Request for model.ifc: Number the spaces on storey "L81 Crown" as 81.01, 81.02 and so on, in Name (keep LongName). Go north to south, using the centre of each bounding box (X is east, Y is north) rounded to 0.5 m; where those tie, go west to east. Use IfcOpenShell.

First a look at what the model holds.

```python
import ifcopenshell
import ifcopenshell.util.element
import ifcopenshell.util.placement

model = ifcopenshell.open("model.ifc")
print(model.schema)
storey = next(s for s in model.by_type("IfcBuildingStorey") if s.Name == "L81 Crown")
spaces = [e for e in ifcopenshell.util.element.get_decomposition(storey) if e.is_a("IfcSpace")]
for e in sorted(spaces, key=lambda e: e.id()):
    origin = ifcopenshell.util.placement.get_local_placement(e.ObjectPlacement)[:3, 3]
    print(e.id(), e.Name, e.LongName, origin.round(2) + 0.0, sep=" | ")
```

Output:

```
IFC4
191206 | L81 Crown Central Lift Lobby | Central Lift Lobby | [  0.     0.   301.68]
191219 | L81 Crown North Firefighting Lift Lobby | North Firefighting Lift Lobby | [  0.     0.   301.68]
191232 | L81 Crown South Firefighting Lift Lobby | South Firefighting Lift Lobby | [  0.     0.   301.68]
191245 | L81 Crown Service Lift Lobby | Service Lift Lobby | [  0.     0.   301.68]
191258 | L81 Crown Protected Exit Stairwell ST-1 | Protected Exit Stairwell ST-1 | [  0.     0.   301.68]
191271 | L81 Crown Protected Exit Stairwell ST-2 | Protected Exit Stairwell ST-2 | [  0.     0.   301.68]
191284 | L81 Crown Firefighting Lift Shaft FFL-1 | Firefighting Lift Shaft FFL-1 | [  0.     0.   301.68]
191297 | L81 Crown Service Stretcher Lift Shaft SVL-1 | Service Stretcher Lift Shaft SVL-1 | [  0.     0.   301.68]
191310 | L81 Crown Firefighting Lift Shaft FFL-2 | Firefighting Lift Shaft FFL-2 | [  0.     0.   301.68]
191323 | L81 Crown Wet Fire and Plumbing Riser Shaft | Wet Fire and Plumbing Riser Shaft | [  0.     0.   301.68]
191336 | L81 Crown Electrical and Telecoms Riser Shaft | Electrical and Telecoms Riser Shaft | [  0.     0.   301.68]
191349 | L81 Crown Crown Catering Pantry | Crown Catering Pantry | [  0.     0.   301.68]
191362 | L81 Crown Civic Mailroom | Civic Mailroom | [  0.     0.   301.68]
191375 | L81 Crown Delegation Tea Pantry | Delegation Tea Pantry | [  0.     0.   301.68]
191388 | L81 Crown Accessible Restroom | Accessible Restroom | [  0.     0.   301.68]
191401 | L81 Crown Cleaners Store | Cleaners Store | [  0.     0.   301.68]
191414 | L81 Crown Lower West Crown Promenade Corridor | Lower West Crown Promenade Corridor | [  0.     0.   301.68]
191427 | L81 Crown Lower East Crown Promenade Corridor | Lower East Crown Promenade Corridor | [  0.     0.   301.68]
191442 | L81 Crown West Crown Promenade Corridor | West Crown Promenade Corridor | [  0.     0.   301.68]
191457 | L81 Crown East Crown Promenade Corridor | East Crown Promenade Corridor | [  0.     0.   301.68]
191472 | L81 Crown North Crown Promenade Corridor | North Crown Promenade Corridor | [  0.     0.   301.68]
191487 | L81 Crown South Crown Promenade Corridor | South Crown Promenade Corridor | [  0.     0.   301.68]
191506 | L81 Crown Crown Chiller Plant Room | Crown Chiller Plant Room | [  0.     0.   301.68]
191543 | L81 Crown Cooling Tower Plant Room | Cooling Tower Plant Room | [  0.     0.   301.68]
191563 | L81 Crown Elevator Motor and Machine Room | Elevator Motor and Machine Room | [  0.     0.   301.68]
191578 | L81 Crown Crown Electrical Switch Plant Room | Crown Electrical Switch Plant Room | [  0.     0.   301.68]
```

```python
import ifcopenshell
import ifcopenshell.geom
import ifcopenshell.util.element
import ifcopenshell.util.shape

model = ifcopenshell.open("model.ifc")
settings = ifcopenshell.geom.settings()
settings.set("use-world-coords", True)


def centre(element):
    shape = ifcopenshell.geom.create_shape(settings, element)
    return ifcopenshell.util.shape.get_bbox_centroid(shape.geometry)


storey = next(s for s in model.by_type("IfcBuildingStorey") if s.Name == "L81 Crown")
spaces = [e for e in ifcopenshell.util.element.get_decomposition(storey) if e.is_a("IfcSpace")]

# Insertion points can sit at a corner or the storey origin, so sort by the geometry (in metres).
centres = {e: centre(e) for e in spaces}
spaces.sort(key=lambda e: (-round(centres[e][1] / 0.5), centres[e][0]))

for i, e in enumerate(spaces, start=1):
    number = f"81.{i:02d}"
    e.Name = number
    print(e.id(), number)

model.write("model-out.ifc")
```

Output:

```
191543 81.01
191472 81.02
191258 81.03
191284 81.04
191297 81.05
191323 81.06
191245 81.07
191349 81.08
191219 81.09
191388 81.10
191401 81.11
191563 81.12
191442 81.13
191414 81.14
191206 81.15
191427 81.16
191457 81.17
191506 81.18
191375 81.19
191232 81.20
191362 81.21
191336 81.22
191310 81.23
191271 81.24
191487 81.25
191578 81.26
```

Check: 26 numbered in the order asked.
